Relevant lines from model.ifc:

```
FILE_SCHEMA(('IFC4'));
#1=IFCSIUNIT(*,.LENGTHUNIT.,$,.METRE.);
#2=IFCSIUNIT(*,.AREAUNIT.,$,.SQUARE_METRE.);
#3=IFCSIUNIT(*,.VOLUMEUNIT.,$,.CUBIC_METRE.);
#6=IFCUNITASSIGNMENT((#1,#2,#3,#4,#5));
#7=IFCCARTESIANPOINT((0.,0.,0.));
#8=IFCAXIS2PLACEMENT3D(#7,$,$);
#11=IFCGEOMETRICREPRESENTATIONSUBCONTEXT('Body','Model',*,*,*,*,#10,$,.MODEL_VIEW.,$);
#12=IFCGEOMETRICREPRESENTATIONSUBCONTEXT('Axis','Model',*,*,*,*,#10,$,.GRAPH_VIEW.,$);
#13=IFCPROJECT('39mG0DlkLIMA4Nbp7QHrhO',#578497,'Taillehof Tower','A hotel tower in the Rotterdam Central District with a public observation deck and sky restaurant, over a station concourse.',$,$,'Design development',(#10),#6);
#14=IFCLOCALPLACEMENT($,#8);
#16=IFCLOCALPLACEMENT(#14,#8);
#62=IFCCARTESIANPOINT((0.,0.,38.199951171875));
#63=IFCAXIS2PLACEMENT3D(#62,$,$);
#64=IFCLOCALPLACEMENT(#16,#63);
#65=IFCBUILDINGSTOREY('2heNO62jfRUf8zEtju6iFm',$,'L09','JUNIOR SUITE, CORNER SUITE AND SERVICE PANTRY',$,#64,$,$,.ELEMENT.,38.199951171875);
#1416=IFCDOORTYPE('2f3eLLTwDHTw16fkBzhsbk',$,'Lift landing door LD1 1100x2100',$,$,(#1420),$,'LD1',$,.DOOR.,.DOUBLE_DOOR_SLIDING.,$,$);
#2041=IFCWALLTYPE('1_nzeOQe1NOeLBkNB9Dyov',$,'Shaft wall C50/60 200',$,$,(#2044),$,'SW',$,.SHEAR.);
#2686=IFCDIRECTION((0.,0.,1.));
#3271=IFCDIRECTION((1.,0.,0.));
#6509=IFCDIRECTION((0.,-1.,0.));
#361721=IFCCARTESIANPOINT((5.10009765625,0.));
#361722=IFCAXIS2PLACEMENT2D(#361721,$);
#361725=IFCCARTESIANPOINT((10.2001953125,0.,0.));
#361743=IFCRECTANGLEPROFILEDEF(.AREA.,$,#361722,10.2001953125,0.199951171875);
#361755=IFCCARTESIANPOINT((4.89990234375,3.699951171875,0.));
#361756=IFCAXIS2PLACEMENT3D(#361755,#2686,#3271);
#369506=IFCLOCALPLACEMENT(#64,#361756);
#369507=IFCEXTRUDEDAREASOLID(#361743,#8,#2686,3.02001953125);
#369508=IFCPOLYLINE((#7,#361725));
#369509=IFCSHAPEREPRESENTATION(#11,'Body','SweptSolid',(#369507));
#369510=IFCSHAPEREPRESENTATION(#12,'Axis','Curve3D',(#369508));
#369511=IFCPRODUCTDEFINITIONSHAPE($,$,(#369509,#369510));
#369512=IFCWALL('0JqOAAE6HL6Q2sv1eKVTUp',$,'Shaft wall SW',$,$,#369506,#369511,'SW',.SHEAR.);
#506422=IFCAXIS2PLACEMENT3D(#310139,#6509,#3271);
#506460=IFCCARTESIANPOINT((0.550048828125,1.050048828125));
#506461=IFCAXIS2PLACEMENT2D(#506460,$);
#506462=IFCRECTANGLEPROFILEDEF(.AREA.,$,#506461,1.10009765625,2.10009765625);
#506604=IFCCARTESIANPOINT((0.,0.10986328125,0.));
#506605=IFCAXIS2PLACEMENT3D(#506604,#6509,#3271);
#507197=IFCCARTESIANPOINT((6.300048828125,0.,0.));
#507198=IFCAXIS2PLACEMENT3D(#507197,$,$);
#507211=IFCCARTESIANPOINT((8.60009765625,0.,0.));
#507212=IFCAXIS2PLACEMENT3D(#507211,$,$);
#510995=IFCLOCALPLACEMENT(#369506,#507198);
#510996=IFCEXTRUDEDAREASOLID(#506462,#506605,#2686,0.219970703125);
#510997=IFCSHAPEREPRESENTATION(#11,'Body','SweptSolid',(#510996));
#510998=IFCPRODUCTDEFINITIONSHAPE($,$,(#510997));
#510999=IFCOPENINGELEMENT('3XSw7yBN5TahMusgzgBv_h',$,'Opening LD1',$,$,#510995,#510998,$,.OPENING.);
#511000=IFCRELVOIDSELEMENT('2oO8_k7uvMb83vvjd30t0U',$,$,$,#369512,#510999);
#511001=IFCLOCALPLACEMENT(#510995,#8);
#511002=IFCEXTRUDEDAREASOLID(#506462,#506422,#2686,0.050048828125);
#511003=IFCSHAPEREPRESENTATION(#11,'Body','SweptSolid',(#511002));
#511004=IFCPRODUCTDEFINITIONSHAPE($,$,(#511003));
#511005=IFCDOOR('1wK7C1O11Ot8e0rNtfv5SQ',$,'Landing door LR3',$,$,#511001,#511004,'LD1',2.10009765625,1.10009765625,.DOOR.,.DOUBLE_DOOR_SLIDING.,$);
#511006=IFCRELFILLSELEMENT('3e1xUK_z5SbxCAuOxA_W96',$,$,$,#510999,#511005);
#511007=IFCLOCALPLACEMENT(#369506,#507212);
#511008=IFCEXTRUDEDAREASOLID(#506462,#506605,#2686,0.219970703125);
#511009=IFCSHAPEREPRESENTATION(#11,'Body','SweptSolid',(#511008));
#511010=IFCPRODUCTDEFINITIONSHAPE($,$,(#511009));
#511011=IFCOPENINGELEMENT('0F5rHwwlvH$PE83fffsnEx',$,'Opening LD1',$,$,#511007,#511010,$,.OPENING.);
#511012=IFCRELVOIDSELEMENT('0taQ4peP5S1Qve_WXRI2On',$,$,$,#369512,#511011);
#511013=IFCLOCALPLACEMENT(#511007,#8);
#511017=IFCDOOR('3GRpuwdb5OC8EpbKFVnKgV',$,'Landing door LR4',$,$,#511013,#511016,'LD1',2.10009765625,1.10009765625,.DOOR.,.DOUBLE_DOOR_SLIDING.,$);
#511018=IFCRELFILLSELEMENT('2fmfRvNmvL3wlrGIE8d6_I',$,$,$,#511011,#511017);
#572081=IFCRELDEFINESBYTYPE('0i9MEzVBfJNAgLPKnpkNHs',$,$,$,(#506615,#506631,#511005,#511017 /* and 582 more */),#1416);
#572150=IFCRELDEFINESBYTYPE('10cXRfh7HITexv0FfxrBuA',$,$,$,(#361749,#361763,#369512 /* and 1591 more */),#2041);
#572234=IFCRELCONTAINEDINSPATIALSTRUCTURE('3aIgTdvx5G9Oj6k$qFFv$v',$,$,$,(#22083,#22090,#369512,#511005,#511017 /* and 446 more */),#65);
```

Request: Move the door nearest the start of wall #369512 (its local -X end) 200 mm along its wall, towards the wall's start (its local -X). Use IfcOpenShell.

```python
import ifcopenshell
import ifcopenshell.api.geometry
import ifcopenshell.util.placement
import ifcopenshell.util.unit

model = ifcopenshell.open("model.ifc")
unit_scale = ifcopenshell.util.unit.calculate_unit_scale(model)

door = model.by_guid("1wK7C1O11Ot8e0rNtfv5SQ")
opening = door.FillsVoids[0].RelatingOpeningElement
wall = opening.VoidsElements[0].RelatingBuildingElement

wall_matrix = ifcopenshell.util.placement.get_local_placement(wall.ObjectPlacement)
shift = wall_matrix[:3, 0] * -0.2 / unit_scale
before = ifcopenshell.util.placement.get_local_placement(door.ObjectPlacement)[:3, 3].copy()

# The door is placed relative to its opening, so it follows when the opening moves.
matrix = ifcopenshell.util.placement.get_local_placement(opening.ObjectPlacement)
matrix[:3, 3] += shift
ifcopenshell.api.geometry.edit_object_placement(
    model, product=opening, matrix=matrix, is_si=False, should_transform_children=True
)

after = ifcopenshell.util.placement.get_local_placement(door.ObjectPlacement)[:3, 3]
print("door moved by", (after - before).round(3) + 0.0)

model.write("model-out.ifc")
```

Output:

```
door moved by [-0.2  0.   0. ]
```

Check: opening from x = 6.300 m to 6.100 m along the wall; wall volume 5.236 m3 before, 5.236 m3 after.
